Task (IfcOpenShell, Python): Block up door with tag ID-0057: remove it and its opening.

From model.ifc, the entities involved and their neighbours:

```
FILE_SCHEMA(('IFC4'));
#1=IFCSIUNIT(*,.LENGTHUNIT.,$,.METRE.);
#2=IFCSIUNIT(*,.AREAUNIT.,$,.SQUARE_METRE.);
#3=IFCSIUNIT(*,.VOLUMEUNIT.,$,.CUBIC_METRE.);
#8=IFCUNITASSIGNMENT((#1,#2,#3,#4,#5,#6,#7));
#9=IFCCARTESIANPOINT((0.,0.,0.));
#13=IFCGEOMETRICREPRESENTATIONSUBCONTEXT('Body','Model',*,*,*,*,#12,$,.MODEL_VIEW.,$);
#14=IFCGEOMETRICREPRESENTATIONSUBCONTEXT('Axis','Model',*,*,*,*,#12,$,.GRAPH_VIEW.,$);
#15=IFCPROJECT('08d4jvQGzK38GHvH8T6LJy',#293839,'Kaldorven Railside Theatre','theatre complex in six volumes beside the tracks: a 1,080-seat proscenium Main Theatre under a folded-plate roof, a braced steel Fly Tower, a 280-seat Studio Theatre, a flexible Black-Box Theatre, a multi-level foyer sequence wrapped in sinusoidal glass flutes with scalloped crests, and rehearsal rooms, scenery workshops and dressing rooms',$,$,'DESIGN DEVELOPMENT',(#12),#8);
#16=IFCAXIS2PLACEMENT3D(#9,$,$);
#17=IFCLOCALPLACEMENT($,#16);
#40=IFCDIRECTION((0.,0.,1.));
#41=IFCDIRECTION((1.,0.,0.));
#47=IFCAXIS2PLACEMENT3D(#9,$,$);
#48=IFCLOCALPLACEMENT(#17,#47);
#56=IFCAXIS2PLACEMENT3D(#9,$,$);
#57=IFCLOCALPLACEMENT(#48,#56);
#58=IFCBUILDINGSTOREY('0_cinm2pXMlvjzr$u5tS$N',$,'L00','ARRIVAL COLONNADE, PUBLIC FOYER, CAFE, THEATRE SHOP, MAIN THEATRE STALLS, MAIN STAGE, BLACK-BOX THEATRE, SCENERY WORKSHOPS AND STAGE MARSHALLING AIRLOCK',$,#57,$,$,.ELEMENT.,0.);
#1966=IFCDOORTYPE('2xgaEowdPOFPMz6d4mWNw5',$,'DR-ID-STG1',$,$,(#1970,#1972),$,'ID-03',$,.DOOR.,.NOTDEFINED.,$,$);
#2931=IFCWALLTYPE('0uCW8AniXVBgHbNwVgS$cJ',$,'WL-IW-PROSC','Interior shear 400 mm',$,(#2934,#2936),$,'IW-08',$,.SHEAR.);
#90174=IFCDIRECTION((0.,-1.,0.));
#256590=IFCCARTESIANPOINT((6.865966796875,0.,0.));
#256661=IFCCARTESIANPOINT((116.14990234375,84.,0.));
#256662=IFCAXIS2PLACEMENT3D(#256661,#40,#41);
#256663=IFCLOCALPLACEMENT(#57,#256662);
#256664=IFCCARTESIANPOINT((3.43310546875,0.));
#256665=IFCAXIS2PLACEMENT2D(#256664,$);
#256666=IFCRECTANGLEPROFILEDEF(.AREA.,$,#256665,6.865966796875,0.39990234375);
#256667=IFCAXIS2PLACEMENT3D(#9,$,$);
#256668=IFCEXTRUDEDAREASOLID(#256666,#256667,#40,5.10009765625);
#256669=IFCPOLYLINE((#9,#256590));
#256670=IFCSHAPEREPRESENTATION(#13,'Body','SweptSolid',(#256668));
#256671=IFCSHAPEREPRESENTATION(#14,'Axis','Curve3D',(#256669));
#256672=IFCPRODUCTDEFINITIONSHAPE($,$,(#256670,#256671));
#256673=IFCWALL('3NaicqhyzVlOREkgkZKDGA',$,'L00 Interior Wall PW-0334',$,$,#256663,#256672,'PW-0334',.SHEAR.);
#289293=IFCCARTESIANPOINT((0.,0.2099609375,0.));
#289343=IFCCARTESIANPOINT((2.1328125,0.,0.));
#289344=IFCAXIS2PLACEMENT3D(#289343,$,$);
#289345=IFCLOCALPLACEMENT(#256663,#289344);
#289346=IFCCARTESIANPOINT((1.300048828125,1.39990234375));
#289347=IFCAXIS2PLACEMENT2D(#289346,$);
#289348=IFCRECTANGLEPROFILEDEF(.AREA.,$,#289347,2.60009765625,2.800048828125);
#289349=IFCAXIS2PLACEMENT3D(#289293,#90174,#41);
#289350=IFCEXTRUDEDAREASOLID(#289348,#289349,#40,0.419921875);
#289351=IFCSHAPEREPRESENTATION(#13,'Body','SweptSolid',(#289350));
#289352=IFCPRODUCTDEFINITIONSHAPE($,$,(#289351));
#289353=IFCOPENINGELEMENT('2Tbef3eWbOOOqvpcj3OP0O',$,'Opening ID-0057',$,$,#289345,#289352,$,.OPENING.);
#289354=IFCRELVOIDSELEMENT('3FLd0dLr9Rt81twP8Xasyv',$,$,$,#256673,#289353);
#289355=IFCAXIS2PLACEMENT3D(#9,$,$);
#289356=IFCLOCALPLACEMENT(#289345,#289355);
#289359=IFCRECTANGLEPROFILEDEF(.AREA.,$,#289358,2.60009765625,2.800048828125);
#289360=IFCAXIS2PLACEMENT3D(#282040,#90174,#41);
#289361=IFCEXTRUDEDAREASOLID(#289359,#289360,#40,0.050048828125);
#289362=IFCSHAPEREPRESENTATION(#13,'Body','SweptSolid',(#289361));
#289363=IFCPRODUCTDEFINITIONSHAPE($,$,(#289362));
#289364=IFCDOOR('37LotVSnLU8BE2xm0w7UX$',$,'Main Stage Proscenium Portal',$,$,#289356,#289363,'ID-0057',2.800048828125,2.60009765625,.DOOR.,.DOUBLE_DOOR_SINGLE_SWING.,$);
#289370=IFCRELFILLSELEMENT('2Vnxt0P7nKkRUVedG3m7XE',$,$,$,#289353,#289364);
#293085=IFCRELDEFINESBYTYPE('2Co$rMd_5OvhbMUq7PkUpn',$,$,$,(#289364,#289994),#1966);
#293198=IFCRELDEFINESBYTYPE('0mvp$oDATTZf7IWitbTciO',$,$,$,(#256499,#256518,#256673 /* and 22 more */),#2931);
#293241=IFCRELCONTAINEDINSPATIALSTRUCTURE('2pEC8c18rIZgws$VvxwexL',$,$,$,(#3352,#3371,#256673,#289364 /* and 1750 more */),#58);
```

```python
import ifcopenshell
import ifcopenshell.api.feature
import ifcopenshell.api.root
import ifcopenshell.geom
import ifcopenshell.util.shape

model = ifcopenshell.open("model.ifc")
settings = ifcopenshell.geom.settings()


def volume(element):
    """Net volume in cubic metres, openings subtracted."""
    shape = ifcopenshell.geom.create_shape(settings, element)
    return ifcopenshell.util.shape.get_volume(shape.geometry)


door = model.by_id(289364)
opening = door.FillsVoids[0].RelatingOpeningElement
wall = opening.VoidsElements[0].RelatingBuildingElement
before = volume(wall)

ifcopenshell.api.root.remove_product(model, product=door)
ifcopenshell.api.feature.remove_feature(model, feature=opening)

after = volume(wall)

print(f"wall volume {before:.3f} -> {after:.3f} m3")

model.write("model_edited.ifc")
```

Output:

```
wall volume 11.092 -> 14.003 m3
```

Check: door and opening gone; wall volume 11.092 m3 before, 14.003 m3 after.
